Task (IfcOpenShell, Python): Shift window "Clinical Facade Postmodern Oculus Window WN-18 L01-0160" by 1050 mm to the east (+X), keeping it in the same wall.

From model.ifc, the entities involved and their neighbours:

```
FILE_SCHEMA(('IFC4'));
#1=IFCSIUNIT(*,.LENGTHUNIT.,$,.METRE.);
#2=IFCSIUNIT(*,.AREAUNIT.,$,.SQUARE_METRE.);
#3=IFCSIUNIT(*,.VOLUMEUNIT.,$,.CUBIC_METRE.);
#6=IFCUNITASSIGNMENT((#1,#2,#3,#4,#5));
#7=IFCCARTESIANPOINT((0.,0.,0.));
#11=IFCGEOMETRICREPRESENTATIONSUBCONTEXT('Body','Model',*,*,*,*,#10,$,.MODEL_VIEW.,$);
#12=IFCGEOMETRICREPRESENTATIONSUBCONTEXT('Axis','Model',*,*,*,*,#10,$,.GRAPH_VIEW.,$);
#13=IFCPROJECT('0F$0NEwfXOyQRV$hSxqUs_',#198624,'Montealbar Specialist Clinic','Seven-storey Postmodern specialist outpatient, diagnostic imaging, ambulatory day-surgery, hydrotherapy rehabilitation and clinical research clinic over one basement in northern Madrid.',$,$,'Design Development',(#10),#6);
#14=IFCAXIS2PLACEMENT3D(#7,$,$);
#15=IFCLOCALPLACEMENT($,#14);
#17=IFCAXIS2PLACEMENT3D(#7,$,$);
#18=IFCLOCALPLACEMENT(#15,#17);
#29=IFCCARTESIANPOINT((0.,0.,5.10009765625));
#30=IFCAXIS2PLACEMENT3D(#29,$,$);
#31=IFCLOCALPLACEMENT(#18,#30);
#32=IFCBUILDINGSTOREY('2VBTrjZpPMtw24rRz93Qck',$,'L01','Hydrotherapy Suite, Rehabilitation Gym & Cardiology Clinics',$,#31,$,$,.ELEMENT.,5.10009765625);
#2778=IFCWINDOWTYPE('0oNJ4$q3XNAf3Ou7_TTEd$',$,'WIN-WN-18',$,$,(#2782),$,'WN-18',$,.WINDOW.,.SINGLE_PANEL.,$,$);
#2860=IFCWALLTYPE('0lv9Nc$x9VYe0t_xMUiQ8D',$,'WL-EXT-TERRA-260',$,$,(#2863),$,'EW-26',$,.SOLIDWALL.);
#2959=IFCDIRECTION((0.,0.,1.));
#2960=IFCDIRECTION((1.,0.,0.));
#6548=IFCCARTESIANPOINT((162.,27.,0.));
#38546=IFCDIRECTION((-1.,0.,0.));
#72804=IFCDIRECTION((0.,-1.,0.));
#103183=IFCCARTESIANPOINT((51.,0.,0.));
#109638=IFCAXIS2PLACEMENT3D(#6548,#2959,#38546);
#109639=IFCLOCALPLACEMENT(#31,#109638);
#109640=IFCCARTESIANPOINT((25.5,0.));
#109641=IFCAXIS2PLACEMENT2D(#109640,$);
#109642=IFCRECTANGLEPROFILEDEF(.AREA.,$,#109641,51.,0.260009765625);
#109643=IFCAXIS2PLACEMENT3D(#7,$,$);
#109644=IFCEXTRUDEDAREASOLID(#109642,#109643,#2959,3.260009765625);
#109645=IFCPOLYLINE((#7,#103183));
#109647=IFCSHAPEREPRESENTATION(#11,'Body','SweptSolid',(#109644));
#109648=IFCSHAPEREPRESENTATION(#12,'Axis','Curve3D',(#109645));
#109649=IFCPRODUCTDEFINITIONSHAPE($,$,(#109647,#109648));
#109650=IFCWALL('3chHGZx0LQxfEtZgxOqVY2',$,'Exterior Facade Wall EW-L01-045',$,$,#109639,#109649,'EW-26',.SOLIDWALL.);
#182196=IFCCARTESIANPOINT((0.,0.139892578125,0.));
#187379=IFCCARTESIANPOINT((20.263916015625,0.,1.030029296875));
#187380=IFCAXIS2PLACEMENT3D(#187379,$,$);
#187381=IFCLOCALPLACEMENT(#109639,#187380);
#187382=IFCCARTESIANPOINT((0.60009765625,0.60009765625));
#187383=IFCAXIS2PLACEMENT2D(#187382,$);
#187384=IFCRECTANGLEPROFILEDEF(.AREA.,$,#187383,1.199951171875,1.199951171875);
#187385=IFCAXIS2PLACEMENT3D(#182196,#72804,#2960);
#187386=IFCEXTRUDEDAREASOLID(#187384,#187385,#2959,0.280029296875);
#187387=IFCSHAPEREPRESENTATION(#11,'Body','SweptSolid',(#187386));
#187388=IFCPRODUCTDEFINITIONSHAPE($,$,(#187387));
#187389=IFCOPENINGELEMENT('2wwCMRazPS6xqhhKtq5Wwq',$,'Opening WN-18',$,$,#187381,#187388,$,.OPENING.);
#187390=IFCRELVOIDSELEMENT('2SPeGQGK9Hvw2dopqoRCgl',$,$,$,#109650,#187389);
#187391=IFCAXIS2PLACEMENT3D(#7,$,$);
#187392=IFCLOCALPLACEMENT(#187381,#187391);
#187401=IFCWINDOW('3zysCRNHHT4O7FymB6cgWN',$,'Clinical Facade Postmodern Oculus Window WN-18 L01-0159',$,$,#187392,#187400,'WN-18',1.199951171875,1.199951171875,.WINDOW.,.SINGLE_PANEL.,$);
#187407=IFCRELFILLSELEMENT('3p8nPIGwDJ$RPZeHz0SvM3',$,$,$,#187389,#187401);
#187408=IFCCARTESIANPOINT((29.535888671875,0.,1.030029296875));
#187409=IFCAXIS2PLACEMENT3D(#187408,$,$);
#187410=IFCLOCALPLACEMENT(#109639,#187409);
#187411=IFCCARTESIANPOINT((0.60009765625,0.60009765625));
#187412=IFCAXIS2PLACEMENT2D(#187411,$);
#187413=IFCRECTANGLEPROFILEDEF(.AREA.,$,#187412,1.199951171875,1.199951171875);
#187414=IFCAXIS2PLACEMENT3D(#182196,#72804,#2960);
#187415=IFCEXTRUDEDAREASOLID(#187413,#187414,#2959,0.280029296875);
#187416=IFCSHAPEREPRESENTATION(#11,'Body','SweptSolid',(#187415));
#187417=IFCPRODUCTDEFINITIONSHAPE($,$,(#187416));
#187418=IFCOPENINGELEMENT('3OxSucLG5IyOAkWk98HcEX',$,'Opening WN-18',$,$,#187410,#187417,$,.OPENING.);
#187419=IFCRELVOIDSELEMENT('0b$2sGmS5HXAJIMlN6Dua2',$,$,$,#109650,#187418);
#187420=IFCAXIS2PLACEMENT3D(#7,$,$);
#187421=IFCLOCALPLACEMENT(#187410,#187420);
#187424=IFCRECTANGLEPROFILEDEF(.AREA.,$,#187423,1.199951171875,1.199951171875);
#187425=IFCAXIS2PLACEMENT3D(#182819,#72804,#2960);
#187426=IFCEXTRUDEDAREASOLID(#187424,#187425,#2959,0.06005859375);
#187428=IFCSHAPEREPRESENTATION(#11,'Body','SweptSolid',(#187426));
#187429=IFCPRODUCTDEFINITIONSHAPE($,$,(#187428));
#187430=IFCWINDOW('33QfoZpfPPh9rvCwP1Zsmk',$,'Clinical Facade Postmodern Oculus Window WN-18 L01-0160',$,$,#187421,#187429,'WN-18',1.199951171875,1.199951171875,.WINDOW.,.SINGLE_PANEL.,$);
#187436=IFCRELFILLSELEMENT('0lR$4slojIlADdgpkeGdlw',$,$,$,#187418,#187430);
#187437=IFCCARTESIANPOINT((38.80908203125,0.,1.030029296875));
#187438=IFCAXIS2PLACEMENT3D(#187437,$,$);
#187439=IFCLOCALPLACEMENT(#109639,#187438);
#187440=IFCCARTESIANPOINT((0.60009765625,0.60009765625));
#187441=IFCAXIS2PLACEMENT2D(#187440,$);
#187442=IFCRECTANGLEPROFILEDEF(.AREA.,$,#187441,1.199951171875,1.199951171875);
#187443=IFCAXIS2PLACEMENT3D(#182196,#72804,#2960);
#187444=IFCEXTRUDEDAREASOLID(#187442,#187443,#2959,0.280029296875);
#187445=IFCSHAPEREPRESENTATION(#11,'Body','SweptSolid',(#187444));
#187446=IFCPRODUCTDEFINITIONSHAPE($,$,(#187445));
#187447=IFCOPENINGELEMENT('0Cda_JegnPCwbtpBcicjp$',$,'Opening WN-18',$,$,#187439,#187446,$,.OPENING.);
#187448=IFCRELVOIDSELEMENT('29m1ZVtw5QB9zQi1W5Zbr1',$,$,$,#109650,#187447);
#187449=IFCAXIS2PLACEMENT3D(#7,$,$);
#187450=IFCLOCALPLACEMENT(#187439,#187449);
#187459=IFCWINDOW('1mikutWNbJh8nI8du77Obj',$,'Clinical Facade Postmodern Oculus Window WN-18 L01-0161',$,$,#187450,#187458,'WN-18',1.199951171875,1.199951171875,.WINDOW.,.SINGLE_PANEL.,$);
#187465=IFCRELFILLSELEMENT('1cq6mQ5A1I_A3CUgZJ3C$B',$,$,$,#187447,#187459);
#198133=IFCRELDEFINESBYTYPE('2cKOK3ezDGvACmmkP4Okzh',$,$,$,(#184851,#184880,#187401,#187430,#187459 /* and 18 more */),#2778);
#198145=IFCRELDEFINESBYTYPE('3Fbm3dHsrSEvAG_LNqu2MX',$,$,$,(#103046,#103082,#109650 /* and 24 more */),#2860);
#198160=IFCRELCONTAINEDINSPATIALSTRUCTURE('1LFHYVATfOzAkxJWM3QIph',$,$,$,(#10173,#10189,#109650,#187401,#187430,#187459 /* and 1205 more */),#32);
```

```python
import ifcopenshell
import ifcopenshell.api.geometry
import ifcopenshell.util.placement

model = ifcopenshell.open("model.ifc")

window = model.by_id(187430)
opening = window.FillsVoids[0].RelatingOpeningElement
wall = opening.VoidsElements[0].RelatingBuildingElement

wall_matrix = ifcopenshell.util.placement.get_local_placement(wall.ObjectPlacement)
shift = wall_matrix[:3, 0] * -1.05
before = ifcopenshell.util.placement.get_local_placement(window.ObjectPlacement)[:3, 3].copy()

# The window is placed relative to its opening, so it follows when the opening moves.
matrix = ifcopenshell.util.placement.get_local_placement(opening.ObjectPlacement)
matrix[:3, 3] += shift
ifcopenshell.api.geometry.edit_object_placement(
    model, product=opening, matrix=matrix, is_si=False, should_transform_children=True
)

after = ifcopenshell.util.placement.get_local_placement(window.ObjectPlacement)[:3, 3]
print("window moved by", (after - before).round(3) + 0.0)

model.write("model_updated.ifc")
```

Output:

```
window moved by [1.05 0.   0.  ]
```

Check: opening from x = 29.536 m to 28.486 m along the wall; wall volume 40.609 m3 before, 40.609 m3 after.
